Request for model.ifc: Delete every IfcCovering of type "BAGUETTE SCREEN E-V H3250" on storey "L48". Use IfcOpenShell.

First a look at what the model holds.

```python
import ifcopenshell
import ifcopenshell.util.element

model = ifcopenshell.open("model.ifc")
print(model.schema)
storey = next(s for s in model.by_type("IfcBuildingStorey") if s.Name == "L48")
coverings = [e for e in ifcopenshell.util.element.get_decomposition(storey) if e.is_a("IfcCovering")]
seen = {}
for e in coverings:
    element_type = ifcopenshell.util.element.get_type(e)
    name = element_type.Name if element_type not in (None, e) else None
    seen[name] = seen.get(name, 0) + 1
for name, count in sorted(seen.items(), key=str):
    print(count, "x", name)
```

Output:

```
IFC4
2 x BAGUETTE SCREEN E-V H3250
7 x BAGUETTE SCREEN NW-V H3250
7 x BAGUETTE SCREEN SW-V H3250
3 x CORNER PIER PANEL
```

```python
import ifcopenshell
import ifcopenshell.api.root
import ifcopenshell.util.element

model = ifcopenshell.open("model.ifc")

storey = next(s for s in model.by_type("IfcBuildingStorey") if s.Name == "L48")
coverings = [e for e in ifcopenshell.util.element.get_decomposition(storey) if e.is_a("IfcCovering")]
targets = [e for e in coverings if (t := ifcopenshell.util.element.get_type(e)) not in (None, e) and t.Name == "BAGUETTE SCREEN E-V H3250"]

for e in targets:
    ifcopenshell.api.root.remove_product(model, product=e)
print(len(targets), "removed")

model.write("model_updated.ifc")
```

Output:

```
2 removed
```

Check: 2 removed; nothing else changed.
